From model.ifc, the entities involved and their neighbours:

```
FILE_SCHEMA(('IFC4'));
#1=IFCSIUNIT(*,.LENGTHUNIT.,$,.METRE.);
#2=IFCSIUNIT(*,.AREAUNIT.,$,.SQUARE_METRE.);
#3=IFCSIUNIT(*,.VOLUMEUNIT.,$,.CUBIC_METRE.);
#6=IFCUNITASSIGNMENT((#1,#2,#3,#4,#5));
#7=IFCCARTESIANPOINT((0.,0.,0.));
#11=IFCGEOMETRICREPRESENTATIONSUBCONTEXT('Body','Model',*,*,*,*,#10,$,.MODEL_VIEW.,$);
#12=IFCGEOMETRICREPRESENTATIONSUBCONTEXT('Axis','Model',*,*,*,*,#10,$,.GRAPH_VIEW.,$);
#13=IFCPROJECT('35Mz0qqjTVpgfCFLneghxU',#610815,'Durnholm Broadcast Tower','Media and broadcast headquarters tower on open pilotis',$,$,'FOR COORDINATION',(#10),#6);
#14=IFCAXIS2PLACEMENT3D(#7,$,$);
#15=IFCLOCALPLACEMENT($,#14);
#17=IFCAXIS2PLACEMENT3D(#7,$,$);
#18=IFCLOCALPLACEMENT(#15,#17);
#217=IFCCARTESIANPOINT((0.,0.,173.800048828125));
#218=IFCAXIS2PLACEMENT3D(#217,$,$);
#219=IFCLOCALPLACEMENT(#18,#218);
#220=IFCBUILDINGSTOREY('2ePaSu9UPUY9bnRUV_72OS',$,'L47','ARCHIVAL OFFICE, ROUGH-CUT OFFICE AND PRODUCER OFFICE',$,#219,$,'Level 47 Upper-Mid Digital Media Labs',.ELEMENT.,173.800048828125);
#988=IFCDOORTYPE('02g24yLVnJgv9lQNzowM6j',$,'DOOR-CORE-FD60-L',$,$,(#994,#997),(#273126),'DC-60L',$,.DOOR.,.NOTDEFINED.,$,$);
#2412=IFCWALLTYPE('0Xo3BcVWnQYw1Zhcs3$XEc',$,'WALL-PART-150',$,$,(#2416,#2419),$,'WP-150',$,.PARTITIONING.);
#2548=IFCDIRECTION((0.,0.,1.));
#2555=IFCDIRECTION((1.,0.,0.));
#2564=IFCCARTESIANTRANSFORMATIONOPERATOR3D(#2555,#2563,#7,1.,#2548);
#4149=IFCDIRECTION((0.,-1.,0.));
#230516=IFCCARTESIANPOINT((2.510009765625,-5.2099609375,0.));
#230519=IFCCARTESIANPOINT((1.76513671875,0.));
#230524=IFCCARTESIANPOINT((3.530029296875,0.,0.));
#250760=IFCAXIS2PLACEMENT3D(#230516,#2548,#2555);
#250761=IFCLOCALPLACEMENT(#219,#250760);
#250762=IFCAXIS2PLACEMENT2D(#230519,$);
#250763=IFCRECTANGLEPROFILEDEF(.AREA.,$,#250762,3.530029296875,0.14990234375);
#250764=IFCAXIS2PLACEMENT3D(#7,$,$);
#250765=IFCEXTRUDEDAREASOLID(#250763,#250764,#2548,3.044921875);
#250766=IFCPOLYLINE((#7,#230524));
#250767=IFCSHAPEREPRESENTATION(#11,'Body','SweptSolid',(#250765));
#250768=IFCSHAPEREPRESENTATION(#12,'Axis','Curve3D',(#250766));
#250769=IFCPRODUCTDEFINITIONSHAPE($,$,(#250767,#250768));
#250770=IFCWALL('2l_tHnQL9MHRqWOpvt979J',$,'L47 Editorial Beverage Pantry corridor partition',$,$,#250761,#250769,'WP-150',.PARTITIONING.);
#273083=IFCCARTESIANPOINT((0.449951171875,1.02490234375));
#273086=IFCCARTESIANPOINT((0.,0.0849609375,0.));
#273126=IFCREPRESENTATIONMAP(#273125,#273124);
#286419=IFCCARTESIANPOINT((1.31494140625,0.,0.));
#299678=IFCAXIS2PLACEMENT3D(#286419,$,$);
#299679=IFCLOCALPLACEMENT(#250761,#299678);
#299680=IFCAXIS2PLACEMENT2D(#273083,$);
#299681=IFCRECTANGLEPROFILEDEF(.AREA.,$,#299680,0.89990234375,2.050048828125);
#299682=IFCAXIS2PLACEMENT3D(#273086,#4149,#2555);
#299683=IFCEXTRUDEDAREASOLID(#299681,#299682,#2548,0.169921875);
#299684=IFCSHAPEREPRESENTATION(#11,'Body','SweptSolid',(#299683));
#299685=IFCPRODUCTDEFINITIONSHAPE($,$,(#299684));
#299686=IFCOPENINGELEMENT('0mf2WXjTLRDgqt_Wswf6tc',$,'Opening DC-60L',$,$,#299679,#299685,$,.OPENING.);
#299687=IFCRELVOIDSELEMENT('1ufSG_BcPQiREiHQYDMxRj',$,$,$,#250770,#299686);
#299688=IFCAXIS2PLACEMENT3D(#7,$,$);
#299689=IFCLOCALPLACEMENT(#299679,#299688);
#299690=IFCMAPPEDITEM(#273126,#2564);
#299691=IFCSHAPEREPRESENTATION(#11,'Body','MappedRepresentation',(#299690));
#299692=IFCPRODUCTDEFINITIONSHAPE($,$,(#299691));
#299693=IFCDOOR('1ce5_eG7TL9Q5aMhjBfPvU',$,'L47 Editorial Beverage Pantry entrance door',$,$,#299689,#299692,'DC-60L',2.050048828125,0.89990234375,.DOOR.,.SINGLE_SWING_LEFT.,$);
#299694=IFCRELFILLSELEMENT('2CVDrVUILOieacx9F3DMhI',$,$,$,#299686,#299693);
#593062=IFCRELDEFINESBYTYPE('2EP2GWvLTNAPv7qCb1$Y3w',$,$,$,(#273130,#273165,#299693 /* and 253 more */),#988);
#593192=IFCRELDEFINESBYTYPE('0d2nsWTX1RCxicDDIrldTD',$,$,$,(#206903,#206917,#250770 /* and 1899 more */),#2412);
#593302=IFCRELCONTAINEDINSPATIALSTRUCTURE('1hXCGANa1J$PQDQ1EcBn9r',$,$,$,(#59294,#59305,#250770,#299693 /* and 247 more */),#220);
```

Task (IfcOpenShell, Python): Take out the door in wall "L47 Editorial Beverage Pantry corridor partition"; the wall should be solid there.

```python
import ifcopenshell
import ifcopenshell.api.feature
import ifcopenshell.api.root
import ifcopenshell.geom
import ifcopenshell.util.shape

model = ifcopenshell.open("model.ifc")
settings = ifcopenshell.geom.settings()


def volume(element):
    """Net volume in cubic metres, openings subtracted."""
    shape = ifcopenshell.geom.create_shape(settings, element)
    return ifcopenshell.util.shape.get_volume(shape.geometry)


door = model.by_guid("1ce5_eG7TL9Q5aMhjBfPvU")
opening = door.FillsVoids[0].RelatingOpeningElement
wall = opening.VoidsElements[0].RelatingBuildingElement
before = volume(wall)

ifcopenshell.api.root.remove_product(model, product=door)
ifcopenshell.api.feature.remove_feature(model, feature=opening)

after = volume(wall)

print(f"wall volume {before:.3f} -> {after:.3f} m3")

model.write("model_updated.ifc")
```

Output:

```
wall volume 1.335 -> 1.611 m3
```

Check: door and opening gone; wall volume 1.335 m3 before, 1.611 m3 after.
